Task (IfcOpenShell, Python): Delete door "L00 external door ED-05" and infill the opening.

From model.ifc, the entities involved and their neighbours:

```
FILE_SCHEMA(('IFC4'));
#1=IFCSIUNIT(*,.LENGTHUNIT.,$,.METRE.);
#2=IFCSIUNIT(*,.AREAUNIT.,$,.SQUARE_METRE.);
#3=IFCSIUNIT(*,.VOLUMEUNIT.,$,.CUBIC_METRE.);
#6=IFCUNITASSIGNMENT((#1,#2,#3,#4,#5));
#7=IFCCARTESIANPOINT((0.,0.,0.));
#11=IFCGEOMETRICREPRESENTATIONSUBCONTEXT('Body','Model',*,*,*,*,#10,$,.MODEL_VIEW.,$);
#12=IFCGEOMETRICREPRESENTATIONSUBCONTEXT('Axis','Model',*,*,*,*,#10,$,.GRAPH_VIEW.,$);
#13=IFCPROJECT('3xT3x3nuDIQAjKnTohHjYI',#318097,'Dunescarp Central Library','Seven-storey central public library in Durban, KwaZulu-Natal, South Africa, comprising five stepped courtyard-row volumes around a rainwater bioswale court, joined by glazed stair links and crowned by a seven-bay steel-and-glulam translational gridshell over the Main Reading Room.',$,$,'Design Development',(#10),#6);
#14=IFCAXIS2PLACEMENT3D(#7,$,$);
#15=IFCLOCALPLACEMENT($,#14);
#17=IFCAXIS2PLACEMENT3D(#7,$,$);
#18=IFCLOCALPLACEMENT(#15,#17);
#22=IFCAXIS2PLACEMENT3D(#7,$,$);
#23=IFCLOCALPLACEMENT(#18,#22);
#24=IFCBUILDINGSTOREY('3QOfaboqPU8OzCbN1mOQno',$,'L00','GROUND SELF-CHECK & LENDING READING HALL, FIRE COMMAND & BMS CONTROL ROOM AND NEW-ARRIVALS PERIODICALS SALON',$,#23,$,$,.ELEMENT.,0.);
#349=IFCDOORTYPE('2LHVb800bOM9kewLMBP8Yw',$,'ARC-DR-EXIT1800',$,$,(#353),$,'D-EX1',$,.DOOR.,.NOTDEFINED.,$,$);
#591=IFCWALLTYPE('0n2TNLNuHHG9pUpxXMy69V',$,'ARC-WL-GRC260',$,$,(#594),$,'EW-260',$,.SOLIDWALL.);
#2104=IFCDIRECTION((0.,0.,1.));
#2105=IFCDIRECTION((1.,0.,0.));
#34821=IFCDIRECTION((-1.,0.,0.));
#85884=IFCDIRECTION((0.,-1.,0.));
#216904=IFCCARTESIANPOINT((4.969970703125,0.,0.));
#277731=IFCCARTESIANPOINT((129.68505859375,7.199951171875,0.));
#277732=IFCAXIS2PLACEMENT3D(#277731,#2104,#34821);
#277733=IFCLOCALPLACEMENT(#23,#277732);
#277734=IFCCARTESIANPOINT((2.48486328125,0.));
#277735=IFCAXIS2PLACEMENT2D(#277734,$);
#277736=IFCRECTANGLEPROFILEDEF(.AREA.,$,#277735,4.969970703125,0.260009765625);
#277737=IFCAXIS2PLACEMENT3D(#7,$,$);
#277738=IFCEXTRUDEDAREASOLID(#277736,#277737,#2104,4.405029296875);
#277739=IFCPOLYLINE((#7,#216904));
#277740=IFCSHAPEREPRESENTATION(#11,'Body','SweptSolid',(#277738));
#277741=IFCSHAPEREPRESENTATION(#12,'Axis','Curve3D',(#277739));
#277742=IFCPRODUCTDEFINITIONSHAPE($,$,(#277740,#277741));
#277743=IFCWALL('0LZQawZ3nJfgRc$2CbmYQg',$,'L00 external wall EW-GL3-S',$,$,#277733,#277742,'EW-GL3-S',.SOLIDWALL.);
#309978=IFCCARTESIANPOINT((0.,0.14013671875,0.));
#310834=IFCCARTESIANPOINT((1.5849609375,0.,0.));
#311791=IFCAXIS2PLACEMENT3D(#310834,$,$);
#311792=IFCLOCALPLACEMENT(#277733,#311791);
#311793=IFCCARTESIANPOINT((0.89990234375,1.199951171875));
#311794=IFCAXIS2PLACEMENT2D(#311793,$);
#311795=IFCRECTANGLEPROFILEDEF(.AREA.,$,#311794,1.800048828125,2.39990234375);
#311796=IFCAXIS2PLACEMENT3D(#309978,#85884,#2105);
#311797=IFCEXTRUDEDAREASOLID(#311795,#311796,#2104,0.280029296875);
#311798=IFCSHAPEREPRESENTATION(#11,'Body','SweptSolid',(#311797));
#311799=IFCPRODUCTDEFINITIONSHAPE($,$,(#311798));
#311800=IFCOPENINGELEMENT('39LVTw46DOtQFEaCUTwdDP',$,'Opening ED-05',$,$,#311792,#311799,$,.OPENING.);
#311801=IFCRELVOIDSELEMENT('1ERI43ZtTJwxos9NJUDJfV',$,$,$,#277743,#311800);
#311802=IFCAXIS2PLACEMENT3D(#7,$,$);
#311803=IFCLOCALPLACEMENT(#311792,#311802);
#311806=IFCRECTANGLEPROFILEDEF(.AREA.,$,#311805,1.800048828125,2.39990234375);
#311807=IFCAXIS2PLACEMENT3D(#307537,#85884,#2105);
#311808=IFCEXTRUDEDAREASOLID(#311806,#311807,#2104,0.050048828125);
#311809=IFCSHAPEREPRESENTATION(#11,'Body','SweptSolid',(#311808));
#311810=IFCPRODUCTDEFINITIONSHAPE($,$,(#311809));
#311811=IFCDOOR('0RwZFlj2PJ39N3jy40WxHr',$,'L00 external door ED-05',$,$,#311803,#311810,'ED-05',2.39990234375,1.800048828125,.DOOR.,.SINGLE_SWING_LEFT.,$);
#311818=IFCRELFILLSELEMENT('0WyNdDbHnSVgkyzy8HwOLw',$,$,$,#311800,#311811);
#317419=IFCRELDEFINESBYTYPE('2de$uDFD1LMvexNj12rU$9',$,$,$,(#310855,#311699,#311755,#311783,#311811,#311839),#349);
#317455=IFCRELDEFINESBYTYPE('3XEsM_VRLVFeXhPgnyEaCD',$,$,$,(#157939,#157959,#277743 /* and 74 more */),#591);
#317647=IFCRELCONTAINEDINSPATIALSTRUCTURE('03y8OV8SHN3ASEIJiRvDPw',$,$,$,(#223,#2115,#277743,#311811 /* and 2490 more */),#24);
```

```python
import ifcopenshell
import ifcopenshell.api.feature
import ifcopenshell.api.root
import ifcopenshell.geom
import ifcopenshell.util.shape

model = ifcopenshell.open("model.ifc")
settings = ifcopenshell.geom.settings()


def volume(element):
    """Net volume in cubic metres, openings subtracted."""
    shape = ifcopenshell.geom.create_shape(settings, element)
    return ifcopenshell.util.shape.get_volume(shape.geometry)


door = model.by_guid("0RwZFlj2PJ39N3jy40WxHr")
opening = door.FillsVoids[0].RelatingOpeningElement
wall = opening.VoidsElements[0].RelatingBuildingElement
before = volume(wall)

ifcopenshell.api.root.remove_product(model, product=door)
ifcopenshell.api.feature.remove_feature(model, feature=opening)

after = volume(wall)

print(f"wall volume {before:.3f} -> {after:.3f} m3")

model.write("model_updated.ifc")
```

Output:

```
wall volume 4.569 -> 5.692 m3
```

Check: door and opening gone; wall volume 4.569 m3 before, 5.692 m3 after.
